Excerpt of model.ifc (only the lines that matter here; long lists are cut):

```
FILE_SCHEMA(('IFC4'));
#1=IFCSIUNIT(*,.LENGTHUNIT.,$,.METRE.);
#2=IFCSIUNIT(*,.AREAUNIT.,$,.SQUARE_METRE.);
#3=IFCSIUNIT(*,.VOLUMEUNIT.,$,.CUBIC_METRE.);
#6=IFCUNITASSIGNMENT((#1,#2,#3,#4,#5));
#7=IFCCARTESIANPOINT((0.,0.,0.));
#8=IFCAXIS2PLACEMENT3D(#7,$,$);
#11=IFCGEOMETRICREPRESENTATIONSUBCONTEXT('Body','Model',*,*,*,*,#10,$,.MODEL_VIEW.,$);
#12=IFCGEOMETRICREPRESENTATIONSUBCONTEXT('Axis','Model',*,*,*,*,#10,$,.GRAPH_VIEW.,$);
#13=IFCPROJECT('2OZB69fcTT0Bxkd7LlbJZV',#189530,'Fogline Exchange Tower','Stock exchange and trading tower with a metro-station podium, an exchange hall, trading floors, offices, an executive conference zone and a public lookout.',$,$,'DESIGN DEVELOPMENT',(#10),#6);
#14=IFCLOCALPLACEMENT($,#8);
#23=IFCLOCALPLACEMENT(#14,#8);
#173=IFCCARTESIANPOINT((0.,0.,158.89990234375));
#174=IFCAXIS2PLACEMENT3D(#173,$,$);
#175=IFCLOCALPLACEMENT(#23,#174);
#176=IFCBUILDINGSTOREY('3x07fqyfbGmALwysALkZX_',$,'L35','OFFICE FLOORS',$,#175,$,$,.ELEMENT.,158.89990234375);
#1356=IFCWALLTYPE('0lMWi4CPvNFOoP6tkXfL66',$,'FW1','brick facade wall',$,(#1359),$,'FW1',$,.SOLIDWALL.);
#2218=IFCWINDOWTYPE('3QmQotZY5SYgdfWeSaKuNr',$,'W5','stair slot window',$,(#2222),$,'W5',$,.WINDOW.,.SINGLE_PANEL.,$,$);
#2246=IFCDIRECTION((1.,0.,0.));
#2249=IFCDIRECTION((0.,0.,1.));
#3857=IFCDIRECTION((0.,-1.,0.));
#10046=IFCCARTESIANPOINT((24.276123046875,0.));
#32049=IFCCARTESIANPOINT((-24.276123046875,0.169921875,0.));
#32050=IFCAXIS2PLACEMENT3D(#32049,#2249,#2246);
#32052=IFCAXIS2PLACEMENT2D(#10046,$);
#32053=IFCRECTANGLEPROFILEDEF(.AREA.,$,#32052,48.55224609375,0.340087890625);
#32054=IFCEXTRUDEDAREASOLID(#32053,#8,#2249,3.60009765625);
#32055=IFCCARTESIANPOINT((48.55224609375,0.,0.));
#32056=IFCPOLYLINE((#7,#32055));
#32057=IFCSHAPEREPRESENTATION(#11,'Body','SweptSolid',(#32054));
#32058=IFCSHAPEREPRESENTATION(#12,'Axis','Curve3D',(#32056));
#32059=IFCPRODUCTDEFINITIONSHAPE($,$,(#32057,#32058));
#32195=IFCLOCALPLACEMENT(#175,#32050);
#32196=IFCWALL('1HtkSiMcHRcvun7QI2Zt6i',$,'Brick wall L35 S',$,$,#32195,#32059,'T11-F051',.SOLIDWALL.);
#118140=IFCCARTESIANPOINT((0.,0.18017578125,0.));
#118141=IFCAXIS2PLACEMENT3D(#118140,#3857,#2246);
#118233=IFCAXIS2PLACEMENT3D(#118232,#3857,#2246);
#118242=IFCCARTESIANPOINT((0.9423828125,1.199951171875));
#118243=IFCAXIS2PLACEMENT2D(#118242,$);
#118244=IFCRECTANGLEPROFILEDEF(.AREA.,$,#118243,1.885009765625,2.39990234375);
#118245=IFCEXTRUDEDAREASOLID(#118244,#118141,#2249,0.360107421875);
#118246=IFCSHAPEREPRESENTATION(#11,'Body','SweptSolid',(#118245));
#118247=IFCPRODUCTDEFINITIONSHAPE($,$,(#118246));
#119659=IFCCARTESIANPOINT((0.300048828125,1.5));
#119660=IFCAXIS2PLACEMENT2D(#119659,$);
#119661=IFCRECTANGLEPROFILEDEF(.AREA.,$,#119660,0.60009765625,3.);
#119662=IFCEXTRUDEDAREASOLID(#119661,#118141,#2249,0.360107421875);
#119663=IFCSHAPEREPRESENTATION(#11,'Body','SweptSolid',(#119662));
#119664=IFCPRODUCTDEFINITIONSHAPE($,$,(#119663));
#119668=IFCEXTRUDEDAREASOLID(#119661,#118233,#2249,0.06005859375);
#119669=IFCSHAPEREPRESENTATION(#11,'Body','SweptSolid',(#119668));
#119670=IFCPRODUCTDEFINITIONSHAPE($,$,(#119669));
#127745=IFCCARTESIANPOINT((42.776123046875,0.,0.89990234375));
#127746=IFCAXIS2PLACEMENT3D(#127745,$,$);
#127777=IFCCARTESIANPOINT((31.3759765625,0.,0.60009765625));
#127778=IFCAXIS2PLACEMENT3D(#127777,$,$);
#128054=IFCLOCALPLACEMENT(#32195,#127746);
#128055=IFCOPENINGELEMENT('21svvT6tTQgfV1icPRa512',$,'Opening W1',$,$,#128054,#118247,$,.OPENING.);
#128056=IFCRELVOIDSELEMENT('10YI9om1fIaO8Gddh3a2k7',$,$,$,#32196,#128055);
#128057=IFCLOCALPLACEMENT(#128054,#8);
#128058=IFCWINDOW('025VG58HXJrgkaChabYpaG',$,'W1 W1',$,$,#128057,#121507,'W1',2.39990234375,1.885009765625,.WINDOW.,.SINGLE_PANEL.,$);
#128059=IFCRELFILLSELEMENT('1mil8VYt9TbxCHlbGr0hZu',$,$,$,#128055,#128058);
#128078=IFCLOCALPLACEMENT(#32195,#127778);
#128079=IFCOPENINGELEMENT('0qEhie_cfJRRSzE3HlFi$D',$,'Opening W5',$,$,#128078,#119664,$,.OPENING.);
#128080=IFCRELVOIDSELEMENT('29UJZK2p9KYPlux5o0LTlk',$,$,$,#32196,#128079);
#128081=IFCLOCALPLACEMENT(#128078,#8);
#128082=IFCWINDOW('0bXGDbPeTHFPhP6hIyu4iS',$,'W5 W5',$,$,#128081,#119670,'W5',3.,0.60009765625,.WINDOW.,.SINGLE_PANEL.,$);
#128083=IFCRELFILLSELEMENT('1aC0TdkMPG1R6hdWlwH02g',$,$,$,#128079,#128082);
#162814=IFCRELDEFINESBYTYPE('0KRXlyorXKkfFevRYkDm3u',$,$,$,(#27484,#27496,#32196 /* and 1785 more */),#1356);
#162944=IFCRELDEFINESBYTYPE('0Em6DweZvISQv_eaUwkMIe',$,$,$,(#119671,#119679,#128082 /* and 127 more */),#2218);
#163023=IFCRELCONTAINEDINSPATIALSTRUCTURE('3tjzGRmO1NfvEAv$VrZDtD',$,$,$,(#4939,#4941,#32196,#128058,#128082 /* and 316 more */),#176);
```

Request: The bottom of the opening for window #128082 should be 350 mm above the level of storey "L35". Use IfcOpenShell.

```python
import numpy as np
import ifcopenshell
import ifcopenshell.api.geometry
import ifcopenshell.geom
import ifcopenshell.util.element
import ifcopenshell.util.placement
import ifcopenshell.util.shape
import ifcopenshell.util.unit

model = ifcopenshell.open("model.ifc")
unit_scale = ifcopenshell.util.unit.calculate_unit_scale(model)

window = model.by_guid("0bXGDbPeTHFPhP6hIyu4iS")
opening = window.FillsVoids[0].RelatingOpeningElement
storey = ifcopenshell.util.element.get_container(window, ifc_class="IfcBuildingStorey")
level = ifcopenshell.util.placement.get_local_placement(storey.ObjectPlacement)[2, 3]

# The opening's origin need not be at the sill, so measure its lowest point.
shape = ifcopenshell.geom.create_shape(ifcopenshell.geom.settings(), opening)
bottom = ifcopenshell.util.shape.get_shape_bottom_elevation(shape, shape.geometry) / unit_scale
dz = level + 0.35 / unit_scale - bottom

shift = np.array([0.0, 0.0, dz])
# The window is placed relative to its opening, so it follows when the opening moves.
matrix = ifcopenshell.util.placement.get_local_placement(opening.ObjectPlacement)
matrix[:3, 3] += shift
ifcopenshell.api.geometry.edit_object_placement(
    model, product=opening, matrix=matrix, is_si=False, should_transform_children=True
)

print(f"moved by {dz * unit_scale:+.3f} m")

model.write("model_rev.ifc")
```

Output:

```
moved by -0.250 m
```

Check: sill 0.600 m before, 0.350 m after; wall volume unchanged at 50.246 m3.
